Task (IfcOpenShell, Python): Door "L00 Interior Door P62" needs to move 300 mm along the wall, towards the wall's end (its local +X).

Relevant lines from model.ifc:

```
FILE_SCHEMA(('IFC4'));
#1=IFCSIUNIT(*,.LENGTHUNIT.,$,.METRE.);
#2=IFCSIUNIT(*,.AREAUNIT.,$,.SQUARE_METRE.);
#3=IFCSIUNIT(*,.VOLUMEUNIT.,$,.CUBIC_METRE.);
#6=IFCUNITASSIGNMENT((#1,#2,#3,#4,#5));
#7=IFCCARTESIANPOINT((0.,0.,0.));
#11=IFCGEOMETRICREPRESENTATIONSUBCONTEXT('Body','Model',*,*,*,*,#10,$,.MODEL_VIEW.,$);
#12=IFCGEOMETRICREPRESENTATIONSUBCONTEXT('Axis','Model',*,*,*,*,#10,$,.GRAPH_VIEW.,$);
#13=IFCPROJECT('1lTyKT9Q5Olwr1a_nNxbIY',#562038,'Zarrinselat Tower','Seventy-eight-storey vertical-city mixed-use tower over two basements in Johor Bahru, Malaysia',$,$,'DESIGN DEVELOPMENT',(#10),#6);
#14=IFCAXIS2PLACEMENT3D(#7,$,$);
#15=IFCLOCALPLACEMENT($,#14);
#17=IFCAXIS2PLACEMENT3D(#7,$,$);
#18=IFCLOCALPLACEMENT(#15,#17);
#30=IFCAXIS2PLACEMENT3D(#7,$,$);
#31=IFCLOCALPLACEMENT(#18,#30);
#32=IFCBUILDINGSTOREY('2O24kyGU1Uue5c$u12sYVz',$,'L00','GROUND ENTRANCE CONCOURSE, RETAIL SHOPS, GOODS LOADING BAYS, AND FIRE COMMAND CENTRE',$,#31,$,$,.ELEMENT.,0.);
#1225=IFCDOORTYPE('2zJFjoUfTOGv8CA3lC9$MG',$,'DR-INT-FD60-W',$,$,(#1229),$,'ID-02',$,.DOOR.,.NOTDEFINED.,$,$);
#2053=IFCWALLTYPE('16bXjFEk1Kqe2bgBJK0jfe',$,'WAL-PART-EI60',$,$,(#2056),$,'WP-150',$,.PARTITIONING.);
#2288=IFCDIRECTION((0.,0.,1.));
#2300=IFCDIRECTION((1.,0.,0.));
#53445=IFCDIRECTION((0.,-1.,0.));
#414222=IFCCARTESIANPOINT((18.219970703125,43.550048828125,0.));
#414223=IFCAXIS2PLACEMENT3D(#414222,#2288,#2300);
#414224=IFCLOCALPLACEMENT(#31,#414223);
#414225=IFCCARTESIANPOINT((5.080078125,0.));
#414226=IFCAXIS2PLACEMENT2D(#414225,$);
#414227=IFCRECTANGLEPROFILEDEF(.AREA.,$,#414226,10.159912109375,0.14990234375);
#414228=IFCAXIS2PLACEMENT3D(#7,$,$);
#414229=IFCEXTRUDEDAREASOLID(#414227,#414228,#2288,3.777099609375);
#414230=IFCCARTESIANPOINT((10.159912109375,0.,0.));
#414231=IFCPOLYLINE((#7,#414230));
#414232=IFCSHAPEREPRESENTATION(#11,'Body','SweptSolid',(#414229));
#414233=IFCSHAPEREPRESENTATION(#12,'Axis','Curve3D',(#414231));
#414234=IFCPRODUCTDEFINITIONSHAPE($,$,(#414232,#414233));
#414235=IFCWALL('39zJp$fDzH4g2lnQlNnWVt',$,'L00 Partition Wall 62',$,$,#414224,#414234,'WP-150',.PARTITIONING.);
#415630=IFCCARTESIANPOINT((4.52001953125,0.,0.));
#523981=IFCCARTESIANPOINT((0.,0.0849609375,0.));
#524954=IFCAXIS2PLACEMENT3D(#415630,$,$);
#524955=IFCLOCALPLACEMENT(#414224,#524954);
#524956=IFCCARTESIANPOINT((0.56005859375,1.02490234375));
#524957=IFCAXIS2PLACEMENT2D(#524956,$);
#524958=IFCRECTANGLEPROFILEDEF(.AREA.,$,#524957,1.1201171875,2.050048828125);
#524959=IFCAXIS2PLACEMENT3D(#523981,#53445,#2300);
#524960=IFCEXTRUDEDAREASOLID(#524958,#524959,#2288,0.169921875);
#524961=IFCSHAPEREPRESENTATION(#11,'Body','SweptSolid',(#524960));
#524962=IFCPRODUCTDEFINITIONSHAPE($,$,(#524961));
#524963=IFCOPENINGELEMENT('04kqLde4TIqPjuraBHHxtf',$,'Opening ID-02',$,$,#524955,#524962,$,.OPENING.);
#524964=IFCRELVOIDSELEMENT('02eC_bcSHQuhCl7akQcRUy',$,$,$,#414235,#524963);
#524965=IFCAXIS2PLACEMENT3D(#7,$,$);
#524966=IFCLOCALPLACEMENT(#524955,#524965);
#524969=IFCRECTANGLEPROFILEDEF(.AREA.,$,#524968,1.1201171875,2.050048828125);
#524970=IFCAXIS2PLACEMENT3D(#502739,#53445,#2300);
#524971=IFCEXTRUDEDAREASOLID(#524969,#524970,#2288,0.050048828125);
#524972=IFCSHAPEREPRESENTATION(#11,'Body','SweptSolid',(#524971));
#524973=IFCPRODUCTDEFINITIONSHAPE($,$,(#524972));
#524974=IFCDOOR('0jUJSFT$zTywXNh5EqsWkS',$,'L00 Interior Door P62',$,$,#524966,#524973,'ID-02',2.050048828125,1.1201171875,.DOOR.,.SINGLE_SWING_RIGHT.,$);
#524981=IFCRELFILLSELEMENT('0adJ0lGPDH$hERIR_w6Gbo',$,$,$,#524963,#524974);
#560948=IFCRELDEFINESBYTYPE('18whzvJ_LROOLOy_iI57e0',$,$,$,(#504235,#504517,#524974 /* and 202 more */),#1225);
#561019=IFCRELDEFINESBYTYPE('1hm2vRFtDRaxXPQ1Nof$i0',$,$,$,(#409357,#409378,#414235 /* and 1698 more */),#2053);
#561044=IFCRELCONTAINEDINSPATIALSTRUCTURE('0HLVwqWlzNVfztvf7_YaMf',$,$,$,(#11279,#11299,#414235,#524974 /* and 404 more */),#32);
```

```python
import ifcopenshell
import ifcopenshell.api.geometry
import ifcopenshell.util.placement

model = ifcopenshell.open("model.ifc")

door = model.by_guid("0jUJSFT$zTywXNh5EqsWkS")
opening = door.FillsVoids[0].RelatingOpeningElement
wall = opening.VoidsElements[0].RelatingBuildingElement

wall_matrix = ifcopenshell.util.placement.get_local_placement(wall.ObjectPlacement)
shift = wall_matrix[:3, 0] * 0.3
before = ifcopenshell.util.placement.get_local_placement(door.ObjectPlacement)[:3, 3].copy()

# The door is placed relative to its opening, so it follows when the opening moves.
matrix = ifcopenshell.util.placement.get_local_placement(opening.ObjectPlacement)
matrix[:3, 3] += shift
ifcopenshell.api.geometry.edit_object_placement(
    model, product=opening, matrix=matrix, is_si=False, should_transform_children=True
)

after = ifcopenshell.util.placement.get_local_placement(door.ObjectPlacement)[:3, 3]
print("door moved by", (after - before).round(3) + 0.0)

model.write("model_rev.ifc")
```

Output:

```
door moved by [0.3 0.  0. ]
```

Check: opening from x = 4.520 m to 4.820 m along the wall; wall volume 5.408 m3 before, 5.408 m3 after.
